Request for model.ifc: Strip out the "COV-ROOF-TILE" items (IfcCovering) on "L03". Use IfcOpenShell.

First a look at what the model holds.

```python
import ifcopenshell
import ifcopenshell.util.element

model = ifcopenshell.open("model.ifc")
print(model.schema)
storey = next(s for s in model.by_type("IfcBuildingStorey") if s.Name == "L03")
coverings = [e for e in ifcopenshell.util.element.get_decomposition(storey) if e.is_a("IfcCovering")]
seen = {}
for e in coverings:
    element_type = ifcopenshell.util.element.get_type(e)
    name = element_type.Name if element_type not in (None, e) else None
    seen[name] = seen.get(name, 0) + 1
for name, count in sorted(seen.items(), key=str):
    print(count, "x", name)
```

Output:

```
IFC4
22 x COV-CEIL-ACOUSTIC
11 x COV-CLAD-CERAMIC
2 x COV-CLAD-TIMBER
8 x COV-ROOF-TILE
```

```python
import ifcopenshell
import ifcopenshell.api.root
import ifcopenshell.util.element

model = ifcopenshell.open("model.ifc")

storey = next(s for s in model.by_type("IfcBuildingStorey") if s.Name == "L03")
coverings = [e for e in ifcopenshell.util.element.get_decomposition(storey) if e.is_a("IfcCovering")]
targets = [e for e in coverings if (t := ifcopenshell.util.element.get_type(e)) not in (None, e) and t.Name == "COV-ROOF-TILE"]

for e in targets:
    ifcopenshell.api.root.remove_product(model, product=e)
print(len(targets), "removed")

model.write("model_updated.ifc")
```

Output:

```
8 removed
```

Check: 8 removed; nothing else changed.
